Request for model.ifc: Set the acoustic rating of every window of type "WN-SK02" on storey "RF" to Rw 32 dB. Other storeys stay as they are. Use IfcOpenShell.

First a look at what the model holds.

```python
import ifcopenshell
import ifcopenshell.util.element

model = ifcopenshell.open("model.ifc")
print(model.schema)
storey = next(s for s in model.by_type("IfcBuildingStorey") if s.Name == "RF")
windows = [e for e in ifcopenshell.util.element.get_decomposition(storey) if e.is_a("IfcWindow")]
seen = {}
for e in windows:
    element_type = ifcopenshell.util.element.get_type(e)
    key = (element_type.Name if element_type != e and element_type else None, ifcopenshell.util.element.get_pset(e, "Pset_WindowCommon", "AcousticRating"))
    seen[key] = seen.get(key, 0) + 1
for (name, value), count in sorted(seen.items(), key=str):
    print(count, "x", name, "|", value)
```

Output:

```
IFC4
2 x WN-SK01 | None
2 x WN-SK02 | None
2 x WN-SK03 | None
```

```python
import ifcopenshell
import ifcopenshell.api.pset
import ifcopenshell.util.element

model = ifcopenshell.open("model.ifc")

storey = next(s for s in model.by_type("IfcBuildingStorey") if s.Name == "RF")
windows = [e for e in ifcopenshell.util.element.get_decomposition(storey) if e.is_a("IfcWindow")]

count = 0
for e in windows:
    element_type = ifcopenshell.util.element.get_type(e)
    if element_type in (None, e) or element_type.Name != "WN-SK02":
        continue
    # add_pset returns the element's existing set when there is one.
    pset = ifcopenshell.api.pset.add_pset(model, product=e, name="Pset_WindowCommon")
    ifcopenshell.api.pset.edit_pset(model, pset=pset, properties={"AcousticRating": "Rw 32 dB"})
    count += 1

print(count, "windows updated")

model.write("model_rev.ifc")
```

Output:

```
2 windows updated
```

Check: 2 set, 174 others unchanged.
